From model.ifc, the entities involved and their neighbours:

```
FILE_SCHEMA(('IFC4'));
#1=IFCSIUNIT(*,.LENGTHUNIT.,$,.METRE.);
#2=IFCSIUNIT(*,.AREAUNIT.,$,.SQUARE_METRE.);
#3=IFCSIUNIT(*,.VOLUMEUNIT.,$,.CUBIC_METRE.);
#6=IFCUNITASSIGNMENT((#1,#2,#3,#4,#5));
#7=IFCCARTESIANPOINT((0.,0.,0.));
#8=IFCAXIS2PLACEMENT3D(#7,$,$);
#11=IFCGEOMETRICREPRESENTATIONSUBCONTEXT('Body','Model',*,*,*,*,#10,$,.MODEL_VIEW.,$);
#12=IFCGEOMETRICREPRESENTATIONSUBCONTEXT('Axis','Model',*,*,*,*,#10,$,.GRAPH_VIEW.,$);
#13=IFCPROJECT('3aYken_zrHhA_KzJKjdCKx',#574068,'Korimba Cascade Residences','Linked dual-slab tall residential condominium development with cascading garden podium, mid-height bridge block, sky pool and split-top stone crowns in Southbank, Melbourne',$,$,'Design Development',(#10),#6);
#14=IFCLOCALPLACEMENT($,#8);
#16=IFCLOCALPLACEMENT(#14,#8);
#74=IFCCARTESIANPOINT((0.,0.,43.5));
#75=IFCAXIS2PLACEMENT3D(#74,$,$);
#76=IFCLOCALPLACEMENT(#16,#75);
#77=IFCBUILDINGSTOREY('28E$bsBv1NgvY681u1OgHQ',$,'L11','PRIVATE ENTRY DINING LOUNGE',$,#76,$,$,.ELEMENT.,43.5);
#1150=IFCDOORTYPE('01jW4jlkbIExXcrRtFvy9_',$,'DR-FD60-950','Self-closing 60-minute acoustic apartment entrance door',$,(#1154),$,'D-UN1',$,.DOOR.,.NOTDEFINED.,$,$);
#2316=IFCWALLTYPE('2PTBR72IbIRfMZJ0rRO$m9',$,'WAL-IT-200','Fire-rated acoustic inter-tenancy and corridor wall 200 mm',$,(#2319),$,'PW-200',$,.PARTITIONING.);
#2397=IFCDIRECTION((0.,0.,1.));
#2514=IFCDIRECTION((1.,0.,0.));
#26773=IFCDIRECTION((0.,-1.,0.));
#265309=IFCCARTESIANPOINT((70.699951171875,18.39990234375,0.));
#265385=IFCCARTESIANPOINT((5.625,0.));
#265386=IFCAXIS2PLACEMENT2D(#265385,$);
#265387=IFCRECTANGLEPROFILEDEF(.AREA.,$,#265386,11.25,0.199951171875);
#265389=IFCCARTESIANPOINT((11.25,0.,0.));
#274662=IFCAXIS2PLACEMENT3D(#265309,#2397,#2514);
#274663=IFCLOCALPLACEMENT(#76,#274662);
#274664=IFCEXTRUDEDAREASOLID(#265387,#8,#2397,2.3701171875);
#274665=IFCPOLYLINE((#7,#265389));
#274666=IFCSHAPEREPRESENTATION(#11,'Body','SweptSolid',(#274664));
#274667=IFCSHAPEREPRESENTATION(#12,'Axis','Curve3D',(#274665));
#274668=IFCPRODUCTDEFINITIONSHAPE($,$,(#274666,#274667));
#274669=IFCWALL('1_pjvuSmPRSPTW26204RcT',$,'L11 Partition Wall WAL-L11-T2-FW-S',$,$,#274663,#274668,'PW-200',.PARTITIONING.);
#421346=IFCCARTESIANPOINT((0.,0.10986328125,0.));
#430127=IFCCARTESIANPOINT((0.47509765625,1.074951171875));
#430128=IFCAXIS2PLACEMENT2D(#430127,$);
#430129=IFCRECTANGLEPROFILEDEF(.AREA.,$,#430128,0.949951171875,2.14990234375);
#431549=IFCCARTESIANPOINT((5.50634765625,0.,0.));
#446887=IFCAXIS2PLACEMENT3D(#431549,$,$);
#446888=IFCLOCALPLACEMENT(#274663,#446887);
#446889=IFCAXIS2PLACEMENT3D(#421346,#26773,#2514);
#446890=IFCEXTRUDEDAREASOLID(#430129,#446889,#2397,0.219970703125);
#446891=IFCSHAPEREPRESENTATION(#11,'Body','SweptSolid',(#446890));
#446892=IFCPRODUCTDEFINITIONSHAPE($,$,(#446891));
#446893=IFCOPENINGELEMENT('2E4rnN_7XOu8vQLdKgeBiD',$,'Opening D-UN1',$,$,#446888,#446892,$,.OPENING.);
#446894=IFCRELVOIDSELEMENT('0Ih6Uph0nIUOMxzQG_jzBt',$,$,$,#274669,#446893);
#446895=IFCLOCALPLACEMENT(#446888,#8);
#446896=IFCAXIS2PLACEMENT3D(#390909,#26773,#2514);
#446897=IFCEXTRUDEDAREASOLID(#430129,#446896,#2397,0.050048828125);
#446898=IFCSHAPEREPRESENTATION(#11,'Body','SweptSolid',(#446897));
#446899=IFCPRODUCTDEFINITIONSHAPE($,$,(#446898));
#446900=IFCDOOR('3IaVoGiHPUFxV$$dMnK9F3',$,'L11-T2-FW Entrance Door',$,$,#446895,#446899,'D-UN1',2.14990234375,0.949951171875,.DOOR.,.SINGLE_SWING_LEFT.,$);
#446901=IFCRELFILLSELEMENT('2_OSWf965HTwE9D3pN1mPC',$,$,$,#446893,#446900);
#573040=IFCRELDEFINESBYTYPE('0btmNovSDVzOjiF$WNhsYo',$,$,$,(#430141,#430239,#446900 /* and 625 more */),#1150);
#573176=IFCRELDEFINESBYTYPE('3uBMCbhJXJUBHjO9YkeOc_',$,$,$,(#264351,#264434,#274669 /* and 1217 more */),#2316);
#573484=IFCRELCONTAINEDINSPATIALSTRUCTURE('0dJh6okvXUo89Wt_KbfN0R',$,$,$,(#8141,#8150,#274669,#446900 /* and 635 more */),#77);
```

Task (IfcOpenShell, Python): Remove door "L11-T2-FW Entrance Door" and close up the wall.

```python
import ifcopenshell
import ifcopenshell.api.feature
import ifcopenshell.api.root
import ifcopenshell.geom
import ifcopenshell.util.shape

model = ifcopenshell.open("model.ifc")
settings = ifcopenshell.geom.settings()


def volume(element):
    """Net volume in cubic metres, openings subtracted."""
    shape = ifcopenshell.geom.create_shape(settings, element)
    return ifcopenshell.util.shape.get_volume(shape.geometry)


door = model.by_guid("3IaVoGiHPUFxV$$dMnK9F3")
opening = door.FillsVoids[0].RelatingOpeningElement
wall = opening.VoidsElements[0].RelatingBuildingElement
before = volume(wall)

ifcopenshell.api.root.remove_product(model, product=door)
ifcopenshell.api.feature.remove_feature(model, feature=opening)

after = volume(wall)

print(f"wall volume {before:.3f} -> {after:.3f} m3")

model.write("model_updated.ifc")
```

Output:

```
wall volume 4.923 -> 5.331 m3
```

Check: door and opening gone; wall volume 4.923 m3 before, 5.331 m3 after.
